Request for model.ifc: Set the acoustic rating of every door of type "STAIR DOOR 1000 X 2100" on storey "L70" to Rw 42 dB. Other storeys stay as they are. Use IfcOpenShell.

First a look at what the model holds.

```python
import ifcopenshell
import ifcopenshell.util.element

model = ifcopenshell.open("model.ifc")
print(model.schema)
storey = next(s for s in model.by_type("IfcBuildingStorey") if s.Name == "L70")
doors = [e for e in ifcopenshell.util.element.get_decomposition(storey) if e.is_a("IfcDoor")]
seen = {}
for e in doors:
    element_type = ifcopenshell.util.element.get_type(e)
    key = (element_type.Name if element_type != e and element_type else None, ifcopenshell.util.element.get_pset(e, "Pset_DoorCommon", "AcousticRating"))
    seen[key] = seen.get(key, 0) + 1
for (name, value), count in sorted(seen.items(), key=str):
    print(count, "x", name, "|", value)
```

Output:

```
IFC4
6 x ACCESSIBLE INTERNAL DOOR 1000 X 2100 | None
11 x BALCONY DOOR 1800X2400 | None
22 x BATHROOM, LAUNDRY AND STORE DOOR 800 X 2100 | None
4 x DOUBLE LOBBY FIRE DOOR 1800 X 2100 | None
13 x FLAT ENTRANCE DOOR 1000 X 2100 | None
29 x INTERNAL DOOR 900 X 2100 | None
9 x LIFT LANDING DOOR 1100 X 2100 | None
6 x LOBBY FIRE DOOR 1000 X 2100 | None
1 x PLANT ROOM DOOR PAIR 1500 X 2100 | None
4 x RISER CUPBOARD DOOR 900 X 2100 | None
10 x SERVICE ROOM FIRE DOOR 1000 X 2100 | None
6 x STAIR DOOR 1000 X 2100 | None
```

```python
import ifcopenshell
import ifcopenshell.api.pset
import ifcopenshell.util.element

model = ifcopenshell.open("model.ifc")

storey = next(s for s in model.by_type("IfcBuildingStorey") if s.Name == "L70")
doors = [e for e in ifcopenshell.util.element.get_decomposition(storey) if e.is_a("IfcDoor")]

count = 0
for e in doors:
    element_type = ifcopenshell.util.element.get_type(e)
    if element_type in (None, e) or element_type.Name != "STAIR DOOR 1000 X 2100":
        continue
    found = ifcopenshell.util.element.get_pset(e, "Pset_DoorCommon", should_inherit=False)
    if found:
        pset = model.by_id(found["id"])
        if len(ifcopenshell.util.element.get_elements_by_pset(pset)) > 1:
            pset = ifcopenshell.api.pset.unshare_pset(model, products=[e], pset=pset)[0]
    else:
        pset = ifcopenshell.api.pset.add_pset(model, product=e, name="Pset_DoorCommon")
    ifcopenshell.api.pset.edit_pset(model, pset=pset, properties={"AcousticRating": "Rw 42 dB"})
    count += 1

print(count, "doors updated")

model.write("model_rev.ifc")
```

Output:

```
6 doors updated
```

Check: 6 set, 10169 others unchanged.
